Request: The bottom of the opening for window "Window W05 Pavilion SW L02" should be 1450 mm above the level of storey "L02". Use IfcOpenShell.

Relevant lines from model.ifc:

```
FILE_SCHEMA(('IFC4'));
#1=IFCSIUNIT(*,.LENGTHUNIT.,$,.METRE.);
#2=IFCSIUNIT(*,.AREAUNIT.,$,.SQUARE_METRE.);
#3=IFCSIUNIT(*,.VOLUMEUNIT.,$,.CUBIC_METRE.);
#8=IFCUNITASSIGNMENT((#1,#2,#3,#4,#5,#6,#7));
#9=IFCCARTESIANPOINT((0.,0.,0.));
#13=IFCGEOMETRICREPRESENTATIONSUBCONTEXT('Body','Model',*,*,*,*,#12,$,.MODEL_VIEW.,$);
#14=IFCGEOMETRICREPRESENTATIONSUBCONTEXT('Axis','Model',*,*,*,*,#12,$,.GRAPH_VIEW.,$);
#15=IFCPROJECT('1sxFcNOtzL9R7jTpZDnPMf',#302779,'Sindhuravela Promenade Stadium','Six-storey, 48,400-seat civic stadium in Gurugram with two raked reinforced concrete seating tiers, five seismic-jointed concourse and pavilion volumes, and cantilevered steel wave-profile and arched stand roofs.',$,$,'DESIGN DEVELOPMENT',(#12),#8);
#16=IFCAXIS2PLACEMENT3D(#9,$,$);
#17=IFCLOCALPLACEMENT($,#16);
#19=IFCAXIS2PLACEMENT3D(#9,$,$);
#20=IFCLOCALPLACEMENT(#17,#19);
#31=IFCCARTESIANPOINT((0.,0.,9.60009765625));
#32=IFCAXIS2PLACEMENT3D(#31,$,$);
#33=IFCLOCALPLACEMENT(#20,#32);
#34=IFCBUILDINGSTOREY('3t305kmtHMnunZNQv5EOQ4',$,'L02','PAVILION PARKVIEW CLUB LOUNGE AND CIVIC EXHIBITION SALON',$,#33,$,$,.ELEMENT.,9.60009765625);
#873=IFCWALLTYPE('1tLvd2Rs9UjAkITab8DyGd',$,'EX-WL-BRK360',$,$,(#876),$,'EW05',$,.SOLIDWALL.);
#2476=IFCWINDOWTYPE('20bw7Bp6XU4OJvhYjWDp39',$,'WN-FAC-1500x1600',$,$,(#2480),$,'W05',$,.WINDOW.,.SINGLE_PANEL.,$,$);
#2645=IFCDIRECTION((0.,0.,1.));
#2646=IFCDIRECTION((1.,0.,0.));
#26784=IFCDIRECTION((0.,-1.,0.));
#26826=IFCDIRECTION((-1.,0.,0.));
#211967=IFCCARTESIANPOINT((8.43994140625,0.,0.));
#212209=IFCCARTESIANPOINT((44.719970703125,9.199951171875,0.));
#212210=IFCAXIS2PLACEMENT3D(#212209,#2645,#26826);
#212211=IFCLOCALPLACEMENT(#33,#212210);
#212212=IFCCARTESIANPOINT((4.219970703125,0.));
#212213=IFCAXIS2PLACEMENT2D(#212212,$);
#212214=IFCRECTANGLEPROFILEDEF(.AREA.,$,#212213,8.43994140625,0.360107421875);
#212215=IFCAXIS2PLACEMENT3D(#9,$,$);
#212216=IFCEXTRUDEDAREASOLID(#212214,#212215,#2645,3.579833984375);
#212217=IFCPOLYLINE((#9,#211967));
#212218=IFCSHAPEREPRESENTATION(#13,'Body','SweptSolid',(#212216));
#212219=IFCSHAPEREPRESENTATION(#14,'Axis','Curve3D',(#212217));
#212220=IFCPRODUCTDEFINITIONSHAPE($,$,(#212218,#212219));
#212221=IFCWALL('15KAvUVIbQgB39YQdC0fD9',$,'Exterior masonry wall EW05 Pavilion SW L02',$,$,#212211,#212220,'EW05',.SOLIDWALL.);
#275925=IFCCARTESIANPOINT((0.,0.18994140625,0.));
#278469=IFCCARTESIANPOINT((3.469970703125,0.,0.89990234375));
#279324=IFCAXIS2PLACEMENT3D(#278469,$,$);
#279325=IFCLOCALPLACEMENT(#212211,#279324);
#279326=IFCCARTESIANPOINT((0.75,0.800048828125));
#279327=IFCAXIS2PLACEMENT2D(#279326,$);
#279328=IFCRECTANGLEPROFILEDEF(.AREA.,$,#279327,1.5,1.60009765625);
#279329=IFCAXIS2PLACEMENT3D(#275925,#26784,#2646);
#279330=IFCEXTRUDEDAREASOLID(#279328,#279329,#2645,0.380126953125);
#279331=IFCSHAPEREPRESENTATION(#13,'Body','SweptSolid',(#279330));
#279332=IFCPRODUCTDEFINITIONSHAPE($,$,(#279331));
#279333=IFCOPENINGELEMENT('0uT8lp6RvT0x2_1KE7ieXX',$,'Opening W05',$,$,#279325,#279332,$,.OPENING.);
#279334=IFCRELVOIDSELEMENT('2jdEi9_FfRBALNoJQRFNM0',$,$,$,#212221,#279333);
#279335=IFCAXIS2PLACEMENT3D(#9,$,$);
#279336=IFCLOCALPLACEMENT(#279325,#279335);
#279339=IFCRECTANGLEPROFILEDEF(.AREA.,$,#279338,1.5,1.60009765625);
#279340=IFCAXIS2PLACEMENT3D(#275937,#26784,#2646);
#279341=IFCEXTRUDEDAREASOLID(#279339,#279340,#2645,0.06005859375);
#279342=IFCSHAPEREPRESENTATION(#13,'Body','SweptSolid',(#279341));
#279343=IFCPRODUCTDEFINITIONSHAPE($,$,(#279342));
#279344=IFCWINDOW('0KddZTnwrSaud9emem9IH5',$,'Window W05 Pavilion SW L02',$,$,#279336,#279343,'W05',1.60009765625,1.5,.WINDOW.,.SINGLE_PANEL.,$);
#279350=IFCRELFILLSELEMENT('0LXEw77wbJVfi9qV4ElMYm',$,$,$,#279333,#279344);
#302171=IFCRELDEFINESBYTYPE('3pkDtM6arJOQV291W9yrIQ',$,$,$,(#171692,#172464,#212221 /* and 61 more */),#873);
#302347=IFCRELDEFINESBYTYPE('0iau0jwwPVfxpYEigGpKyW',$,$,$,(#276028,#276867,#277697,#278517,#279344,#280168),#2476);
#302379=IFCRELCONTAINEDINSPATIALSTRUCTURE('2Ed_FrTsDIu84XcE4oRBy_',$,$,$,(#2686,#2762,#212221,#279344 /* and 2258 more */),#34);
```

```python
import numpy as np
import ifcopenshell
import ifcopenshell.api.geometry
import ifcopenshell.geom
import ifcopenshell.util.element
import ifcopenshell.util.placement
import ifcopenshell.util.shape
import ifcopenshell.util.unit

model = ifcopenshell.open("model.ifc")
unit_scale = ifcopenshell.util.unit.calculate_unit_scale(model)

window = model.by_id(279344)
opening = window.FillsVoids[0].RelatingOpeningElement
storey = ifcopenshell.util.element.get_container(window, ifc_class="IfcBuildingStorey")
level = ifcopenshell.util.placement.get_local_placement(storey.ObjectPlacement)[2, 3]

# The opening's origin need not be at the sill, so measure its lowest point.
shape = ifcopenshell.geom.create_shape(ifcopenshell.geom.settings(), opening)
bottom = ifcopenshell.util.shape.get_shape_bottom_elevation(shape, shape.geometry) / unit_scale
dz = level + 1.45 / unit_scale - bottom

shift = np.array([0.0, 0.0, dz])
# The window is placed relative to its opening, so it follows when the opening moves.
matrix = ifcopenshell.util.placement.get_local_placement(opening.ObjectPlacement)
matrix[:3, 3] += shift
ifcopenshell.api.geometry.edit_object_placement(
    model, product=opening, matrix=matrix, is_si=False, should_transform_children=True
)

print(f"moved by {dz * unit_scale:+.3f} m")

model.write("model_v2.ifc")
```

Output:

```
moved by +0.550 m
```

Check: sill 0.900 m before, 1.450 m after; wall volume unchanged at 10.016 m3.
